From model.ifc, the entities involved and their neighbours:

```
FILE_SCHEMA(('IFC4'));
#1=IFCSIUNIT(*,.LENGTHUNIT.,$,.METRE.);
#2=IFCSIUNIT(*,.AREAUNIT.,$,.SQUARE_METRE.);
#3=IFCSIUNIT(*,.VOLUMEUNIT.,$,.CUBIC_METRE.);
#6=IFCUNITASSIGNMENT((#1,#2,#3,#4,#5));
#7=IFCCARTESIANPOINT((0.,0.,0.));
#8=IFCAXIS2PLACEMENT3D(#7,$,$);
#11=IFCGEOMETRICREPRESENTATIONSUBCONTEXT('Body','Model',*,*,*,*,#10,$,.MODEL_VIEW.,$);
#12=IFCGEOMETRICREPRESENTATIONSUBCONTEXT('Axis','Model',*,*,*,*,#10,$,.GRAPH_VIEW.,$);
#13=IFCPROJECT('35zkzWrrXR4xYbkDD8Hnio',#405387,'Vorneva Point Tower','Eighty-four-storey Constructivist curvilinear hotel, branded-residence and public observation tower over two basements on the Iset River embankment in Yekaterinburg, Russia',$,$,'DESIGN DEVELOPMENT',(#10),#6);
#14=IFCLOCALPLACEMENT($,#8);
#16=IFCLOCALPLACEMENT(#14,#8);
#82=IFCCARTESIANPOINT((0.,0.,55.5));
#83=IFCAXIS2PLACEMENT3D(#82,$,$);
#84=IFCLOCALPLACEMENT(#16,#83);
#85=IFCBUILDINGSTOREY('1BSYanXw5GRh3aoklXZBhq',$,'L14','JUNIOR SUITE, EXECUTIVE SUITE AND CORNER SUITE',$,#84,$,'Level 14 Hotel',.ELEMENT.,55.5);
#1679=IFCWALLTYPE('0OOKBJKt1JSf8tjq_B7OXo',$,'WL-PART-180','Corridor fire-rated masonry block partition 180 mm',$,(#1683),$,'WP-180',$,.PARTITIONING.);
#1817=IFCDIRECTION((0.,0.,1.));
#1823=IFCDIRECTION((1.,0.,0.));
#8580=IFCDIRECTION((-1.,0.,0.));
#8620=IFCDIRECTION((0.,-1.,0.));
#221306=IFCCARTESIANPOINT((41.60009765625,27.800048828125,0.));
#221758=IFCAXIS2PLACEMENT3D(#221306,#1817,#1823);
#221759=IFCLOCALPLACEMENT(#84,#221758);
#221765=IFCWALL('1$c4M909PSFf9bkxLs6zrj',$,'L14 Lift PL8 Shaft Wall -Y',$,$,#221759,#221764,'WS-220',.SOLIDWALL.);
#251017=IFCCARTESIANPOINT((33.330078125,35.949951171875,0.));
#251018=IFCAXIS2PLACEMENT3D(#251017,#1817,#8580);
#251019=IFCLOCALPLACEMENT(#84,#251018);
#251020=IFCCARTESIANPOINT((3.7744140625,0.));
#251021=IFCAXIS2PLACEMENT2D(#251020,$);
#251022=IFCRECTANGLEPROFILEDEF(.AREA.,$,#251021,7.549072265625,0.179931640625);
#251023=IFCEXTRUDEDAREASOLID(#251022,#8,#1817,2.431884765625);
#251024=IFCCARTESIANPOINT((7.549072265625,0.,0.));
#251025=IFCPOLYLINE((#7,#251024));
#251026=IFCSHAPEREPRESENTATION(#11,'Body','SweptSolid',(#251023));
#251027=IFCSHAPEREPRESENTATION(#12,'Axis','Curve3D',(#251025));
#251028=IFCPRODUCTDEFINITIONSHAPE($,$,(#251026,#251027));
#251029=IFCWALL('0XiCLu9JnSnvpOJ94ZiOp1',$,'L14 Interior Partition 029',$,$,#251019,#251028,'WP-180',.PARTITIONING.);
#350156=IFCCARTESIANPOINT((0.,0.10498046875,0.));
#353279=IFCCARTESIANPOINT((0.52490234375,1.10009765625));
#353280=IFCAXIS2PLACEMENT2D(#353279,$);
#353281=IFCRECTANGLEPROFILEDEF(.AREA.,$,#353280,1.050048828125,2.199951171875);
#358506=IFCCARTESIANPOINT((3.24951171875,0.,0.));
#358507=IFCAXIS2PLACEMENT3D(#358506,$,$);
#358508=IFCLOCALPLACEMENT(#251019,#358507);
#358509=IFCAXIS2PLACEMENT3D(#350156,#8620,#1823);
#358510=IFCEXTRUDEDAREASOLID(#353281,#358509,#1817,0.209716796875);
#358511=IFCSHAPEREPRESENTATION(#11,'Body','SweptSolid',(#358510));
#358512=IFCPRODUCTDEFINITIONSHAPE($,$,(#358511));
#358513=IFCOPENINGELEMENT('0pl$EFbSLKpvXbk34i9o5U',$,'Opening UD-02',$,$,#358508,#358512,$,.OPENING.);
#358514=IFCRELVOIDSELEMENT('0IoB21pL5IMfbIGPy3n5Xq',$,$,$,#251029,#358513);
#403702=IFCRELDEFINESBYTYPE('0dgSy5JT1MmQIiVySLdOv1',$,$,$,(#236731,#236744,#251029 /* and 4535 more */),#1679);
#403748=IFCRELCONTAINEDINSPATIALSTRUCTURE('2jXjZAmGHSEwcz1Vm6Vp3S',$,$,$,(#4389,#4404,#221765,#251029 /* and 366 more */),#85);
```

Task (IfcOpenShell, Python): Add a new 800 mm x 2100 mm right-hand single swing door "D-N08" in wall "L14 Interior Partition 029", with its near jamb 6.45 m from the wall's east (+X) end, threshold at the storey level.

```python
import numpy as np
import ifcopenshell
import ifcopenshell.api.feature
import ifcopenshell.api.geometry
import ifcopenshell.api.root
import ifcopenshell.api.spatial
import ifcopenshell.geom
import ifcopenshell.util.element
import ifcopenshell.util.placement
import ifcopenshell.util.representation
import ifcopenshell.util.shape
import ifcopenshell.util.unit

model = ifcopenshell.open("model.ifc")
unit_scale = ifcopenshell.util.unit.calculate_unit_scale(model)
settings = ifcopenshell.geom.settings()


def volume(element):
    """Net volume in cubic metres, openings subtracted."""
    shape = ifcopenshell.geom.create_shape(settings, element)
    return ifcopenshell.util.shape.get_volume(shape.geometry)


wall = model.by_guid("0XiCLu9JnSnvpOJ94ZiOp1")
storey = ifcopenshell.util.element.get_container(wall, ifc_class="IfcBuildingStorey")
context = ifcopenshell.util.representation.get_context(model, "Model", "Body", "MODEL_VIEW")
before = volume(wall)

width, height, from_end, sill = 0.8, 2.1, 6.45, 0.0  # metres

# The wall runs along its own X axis, and the end named is its -X end.
wall_shape = ifcopenshell.geom.create_shape(settings, wall)
x, y, z = ifcopenshell.util.shape.get_vertices(wall_shape.geometry).T
start = x.min() + from_end
face, thickness = float(y.min()), float(y.max() - y.min())
wall_matrix = ifcopenshell.util.placement.get_local_placement(wall.ObjectPlacement)
level = ifcopenshell.util.placement.get_local_placement(storey.ObjectPlacement)[2, 3]


def in_wall(x, y):
    """Placement at x, y metres in the wall's axes, at sill height."""
    matrix = wall_matrix.copy()
    matrix[:, 3] = wall_matrix @ np.array([x / unit_scale, y / unit_scale, 0.0, 1.0])
    matrix[2, 3] = level + sill / unit_scale
    return matrix


# Opening: a box that overshoots both wall faces by 50 mm.
opening = ifcopenshell.api.root.create_entity(model, ifc_class="IfcOpeningElement", predefined_type="OPENING")
box = ifcopenshell.api.geometry.add_wall_representation(
    model, context=context, length=width, height=height, thickness=thickness + 0.1
)
ifcopenshell.api.geometry.assign_representation(model, product=opening, representation=box)
ifcopenshell.api.geometry.edit_object_placement(model, product=opening, matrix=in_wall(start, face - 0.05), is_si=False)
ifcopenshell.api.feature.add_feature(model, feature=opening, element=wall)

door = ifcopenshell.api.root.create_entity(model, ifc_class="IfcDoor", name="D-N08", predefined_type="DOOR")
door.OverallWidth, door.OverallHeight = width / unit_scale, height / unit_scale
door.OperationType = "SINGLE_SWING_RIGHT"
body = ifcopenshell.api.geometry.add_door_representation(
    model,
    context=context,
    overall_width=door.OverallWidth,
    overall_height=door.OverallHeight,
    operation_type="SINGLE_SWING_RIGHT",
    lining_properties={"LiningDepth": thickness / unit_scale, "ThresholdDepth": thickness / unit_scale},
)
ifcopenshell.api.geometry.assign_representation(model, product=door, representation=body)
ifcopenshell.api.spatial.assign_container(model, products=[door], relating_structure=storey)
ifcopenshell.api.feature.add_filling(model, opening=opening, element=door)

# The lining spans the wall, so the door starts at the wall face.
ifcopenshell.api.geometry.edit_object_placement(model, product=door, matrix=in_wall(start, face), is_si=False)

after = volume(wall)

print(f"wall volume {before:.3f} -> {after:.3f} m3")

model.write("model_edited.ifc")
```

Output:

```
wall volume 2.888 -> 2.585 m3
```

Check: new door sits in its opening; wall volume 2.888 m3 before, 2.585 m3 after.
